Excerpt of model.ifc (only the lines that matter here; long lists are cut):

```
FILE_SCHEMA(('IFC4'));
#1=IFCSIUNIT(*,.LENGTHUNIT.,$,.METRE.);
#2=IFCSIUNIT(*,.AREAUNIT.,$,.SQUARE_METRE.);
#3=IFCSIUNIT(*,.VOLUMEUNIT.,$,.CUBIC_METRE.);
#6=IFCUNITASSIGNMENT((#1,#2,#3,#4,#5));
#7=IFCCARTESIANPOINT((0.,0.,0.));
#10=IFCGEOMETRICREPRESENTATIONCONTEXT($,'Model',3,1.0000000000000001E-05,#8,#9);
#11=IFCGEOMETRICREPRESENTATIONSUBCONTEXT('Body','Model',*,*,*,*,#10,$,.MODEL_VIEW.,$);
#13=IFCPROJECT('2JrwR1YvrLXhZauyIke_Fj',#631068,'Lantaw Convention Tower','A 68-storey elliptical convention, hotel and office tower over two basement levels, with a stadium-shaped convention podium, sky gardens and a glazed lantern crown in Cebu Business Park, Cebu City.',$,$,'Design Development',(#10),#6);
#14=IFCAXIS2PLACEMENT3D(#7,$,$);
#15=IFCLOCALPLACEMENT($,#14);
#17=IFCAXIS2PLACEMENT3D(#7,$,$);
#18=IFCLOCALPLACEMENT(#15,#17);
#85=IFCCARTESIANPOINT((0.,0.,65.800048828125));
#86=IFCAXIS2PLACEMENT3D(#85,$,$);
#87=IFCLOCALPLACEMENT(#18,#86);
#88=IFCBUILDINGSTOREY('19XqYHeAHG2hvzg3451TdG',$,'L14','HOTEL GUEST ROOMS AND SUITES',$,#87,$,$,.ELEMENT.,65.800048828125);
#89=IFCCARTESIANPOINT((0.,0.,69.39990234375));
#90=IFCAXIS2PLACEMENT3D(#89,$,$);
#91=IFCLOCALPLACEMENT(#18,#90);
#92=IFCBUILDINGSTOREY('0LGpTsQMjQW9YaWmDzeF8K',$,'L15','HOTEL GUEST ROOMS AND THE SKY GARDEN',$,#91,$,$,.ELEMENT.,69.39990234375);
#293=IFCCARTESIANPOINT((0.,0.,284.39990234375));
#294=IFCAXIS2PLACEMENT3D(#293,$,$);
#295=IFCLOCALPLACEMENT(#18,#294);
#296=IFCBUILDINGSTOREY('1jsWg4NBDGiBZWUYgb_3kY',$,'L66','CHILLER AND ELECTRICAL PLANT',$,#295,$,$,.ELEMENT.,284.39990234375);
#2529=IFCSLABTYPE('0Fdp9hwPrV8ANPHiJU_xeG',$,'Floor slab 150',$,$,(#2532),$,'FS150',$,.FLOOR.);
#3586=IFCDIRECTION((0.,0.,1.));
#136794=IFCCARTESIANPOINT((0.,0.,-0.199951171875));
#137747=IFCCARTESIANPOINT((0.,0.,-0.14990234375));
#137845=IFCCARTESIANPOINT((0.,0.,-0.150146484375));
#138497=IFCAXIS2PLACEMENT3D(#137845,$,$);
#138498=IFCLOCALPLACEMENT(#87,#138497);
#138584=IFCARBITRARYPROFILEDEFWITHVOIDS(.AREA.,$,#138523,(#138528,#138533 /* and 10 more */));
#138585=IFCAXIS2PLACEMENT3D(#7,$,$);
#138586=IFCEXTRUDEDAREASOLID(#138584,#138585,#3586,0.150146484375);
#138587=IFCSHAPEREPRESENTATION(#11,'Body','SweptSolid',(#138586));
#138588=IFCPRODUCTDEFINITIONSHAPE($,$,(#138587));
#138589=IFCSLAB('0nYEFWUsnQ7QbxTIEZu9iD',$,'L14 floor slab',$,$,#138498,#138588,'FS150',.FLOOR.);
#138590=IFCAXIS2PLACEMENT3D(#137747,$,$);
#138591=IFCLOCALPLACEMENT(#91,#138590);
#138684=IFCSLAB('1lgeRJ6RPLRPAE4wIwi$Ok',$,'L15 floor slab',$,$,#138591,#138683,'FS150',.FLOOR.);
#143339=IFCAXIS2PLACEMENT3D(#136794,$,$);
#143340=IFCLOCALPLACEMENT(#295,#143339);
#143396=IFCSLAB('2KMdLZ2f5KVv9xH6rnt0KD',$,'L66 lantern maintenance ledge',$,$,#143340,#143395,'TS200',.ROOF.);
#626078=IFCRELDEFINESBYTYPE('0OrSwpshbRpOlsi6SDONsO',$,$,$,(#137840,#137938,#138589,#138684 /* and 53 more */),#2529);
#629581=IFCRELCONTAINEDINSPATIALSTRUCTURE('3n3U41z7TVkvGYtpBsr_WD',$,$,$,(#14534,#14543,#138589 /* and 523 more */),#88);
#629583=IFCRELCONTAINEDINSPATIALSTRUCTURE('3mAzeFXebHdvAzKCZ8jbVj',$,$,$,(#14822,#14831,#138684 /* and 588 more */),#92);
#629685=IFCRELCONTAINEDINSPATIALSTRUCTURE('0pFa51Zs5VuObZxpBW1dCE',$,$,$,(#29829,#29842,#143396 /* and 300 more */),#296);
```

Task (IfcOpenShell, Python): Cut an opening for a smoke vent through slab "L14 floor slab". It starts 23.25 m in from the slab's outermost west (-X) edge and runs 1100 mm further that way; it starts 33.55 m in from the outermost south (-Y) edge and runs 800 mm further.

```python
import numpy as np
import ifcopenshell
import ifcopenshell.api.feature
import ifcopenshell.api.geometry
import ifcopenshell.api.root
import ifcopenshell.geom
import ifcopenshell.util.placement
import ifcopenshell.util.representation
import ifcopenshell.util.shape
import ifcopenshell.util.unit

model = ifcopenshell.open("model.ifc")
unit_scale = ifcopenshell.util.unit.calculate_unit_scale(model)
settings = ifcopenshell.geom.settings()


def volume(element):
    """Net volume in cubic metres, openings subtracted."""
    shape = ifcopenshell.geom.create_shape(settings, element)
    return ifcopenshell.util.shape.get_volume(shape.geometry)


slab = model.by_guid("0nYEFWUsnQ7QbxTIEZu9iD")
before = volume(slab)

# Extent in the slab's own axes, in metres. The edges named are its -X and -Y sides.
slab_shape = ifcopenshell.geom.create_shape(settings, slab)
vertices = ifcopenshell.util.shape.get_vertices(slab_shape.geometry)
x_min, y_min, bottom = vertices.min(axis=0)
top = vertices[:, 2].max()

opening = ifcopenshell.api.root.create_entity(model, ifc_class="IfcOpeningElement", name="Smoke vent opening", predefined_type="OPENING")
context = ifcopenshell.util.representation.get_context(model, "Model", "Body", "MODEL_VIEW")
width, depth = 1.1, 0.8
outline = [(0.0, 0.0), (width, 0.0), (width, depth), (0.0, depth), (0.0, 0.0)]
# Overshoot both faces by 50 mm so the cut is clean.
shape = ifcopenshell.api.geometry.add_slab_representation(
    model, context=context, depth=top - bottom + 0.1, polyline=outline
)
ifcopenshell.api.geometry.assign_representation(model, product=opening, representation=shape)

matrix = ifcopenshell.util.placement.get_local_placement(slab.ObjectPlacement)
matrix[:, 3] = matrix @ np.append(np.array([x_min + 23.25, y_min + 33.55, bottom - 0.05]) / unit_scale, 1.0)
ifcopenshell.api.geometry.edit_object_placement(model, product=opening, matrix=matrix, is_si=False)
ifcopenshell.api.feature.add_feature(model, feature=opening, element=slab)

after = volume(slab)

print(f"slab volume {before:.3f} -> {after:.3f} m3")

model.write("model_updated.ifc")
```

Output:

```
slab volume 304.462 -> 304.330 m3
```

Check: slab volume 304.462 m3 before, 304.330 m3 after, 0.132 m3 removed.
